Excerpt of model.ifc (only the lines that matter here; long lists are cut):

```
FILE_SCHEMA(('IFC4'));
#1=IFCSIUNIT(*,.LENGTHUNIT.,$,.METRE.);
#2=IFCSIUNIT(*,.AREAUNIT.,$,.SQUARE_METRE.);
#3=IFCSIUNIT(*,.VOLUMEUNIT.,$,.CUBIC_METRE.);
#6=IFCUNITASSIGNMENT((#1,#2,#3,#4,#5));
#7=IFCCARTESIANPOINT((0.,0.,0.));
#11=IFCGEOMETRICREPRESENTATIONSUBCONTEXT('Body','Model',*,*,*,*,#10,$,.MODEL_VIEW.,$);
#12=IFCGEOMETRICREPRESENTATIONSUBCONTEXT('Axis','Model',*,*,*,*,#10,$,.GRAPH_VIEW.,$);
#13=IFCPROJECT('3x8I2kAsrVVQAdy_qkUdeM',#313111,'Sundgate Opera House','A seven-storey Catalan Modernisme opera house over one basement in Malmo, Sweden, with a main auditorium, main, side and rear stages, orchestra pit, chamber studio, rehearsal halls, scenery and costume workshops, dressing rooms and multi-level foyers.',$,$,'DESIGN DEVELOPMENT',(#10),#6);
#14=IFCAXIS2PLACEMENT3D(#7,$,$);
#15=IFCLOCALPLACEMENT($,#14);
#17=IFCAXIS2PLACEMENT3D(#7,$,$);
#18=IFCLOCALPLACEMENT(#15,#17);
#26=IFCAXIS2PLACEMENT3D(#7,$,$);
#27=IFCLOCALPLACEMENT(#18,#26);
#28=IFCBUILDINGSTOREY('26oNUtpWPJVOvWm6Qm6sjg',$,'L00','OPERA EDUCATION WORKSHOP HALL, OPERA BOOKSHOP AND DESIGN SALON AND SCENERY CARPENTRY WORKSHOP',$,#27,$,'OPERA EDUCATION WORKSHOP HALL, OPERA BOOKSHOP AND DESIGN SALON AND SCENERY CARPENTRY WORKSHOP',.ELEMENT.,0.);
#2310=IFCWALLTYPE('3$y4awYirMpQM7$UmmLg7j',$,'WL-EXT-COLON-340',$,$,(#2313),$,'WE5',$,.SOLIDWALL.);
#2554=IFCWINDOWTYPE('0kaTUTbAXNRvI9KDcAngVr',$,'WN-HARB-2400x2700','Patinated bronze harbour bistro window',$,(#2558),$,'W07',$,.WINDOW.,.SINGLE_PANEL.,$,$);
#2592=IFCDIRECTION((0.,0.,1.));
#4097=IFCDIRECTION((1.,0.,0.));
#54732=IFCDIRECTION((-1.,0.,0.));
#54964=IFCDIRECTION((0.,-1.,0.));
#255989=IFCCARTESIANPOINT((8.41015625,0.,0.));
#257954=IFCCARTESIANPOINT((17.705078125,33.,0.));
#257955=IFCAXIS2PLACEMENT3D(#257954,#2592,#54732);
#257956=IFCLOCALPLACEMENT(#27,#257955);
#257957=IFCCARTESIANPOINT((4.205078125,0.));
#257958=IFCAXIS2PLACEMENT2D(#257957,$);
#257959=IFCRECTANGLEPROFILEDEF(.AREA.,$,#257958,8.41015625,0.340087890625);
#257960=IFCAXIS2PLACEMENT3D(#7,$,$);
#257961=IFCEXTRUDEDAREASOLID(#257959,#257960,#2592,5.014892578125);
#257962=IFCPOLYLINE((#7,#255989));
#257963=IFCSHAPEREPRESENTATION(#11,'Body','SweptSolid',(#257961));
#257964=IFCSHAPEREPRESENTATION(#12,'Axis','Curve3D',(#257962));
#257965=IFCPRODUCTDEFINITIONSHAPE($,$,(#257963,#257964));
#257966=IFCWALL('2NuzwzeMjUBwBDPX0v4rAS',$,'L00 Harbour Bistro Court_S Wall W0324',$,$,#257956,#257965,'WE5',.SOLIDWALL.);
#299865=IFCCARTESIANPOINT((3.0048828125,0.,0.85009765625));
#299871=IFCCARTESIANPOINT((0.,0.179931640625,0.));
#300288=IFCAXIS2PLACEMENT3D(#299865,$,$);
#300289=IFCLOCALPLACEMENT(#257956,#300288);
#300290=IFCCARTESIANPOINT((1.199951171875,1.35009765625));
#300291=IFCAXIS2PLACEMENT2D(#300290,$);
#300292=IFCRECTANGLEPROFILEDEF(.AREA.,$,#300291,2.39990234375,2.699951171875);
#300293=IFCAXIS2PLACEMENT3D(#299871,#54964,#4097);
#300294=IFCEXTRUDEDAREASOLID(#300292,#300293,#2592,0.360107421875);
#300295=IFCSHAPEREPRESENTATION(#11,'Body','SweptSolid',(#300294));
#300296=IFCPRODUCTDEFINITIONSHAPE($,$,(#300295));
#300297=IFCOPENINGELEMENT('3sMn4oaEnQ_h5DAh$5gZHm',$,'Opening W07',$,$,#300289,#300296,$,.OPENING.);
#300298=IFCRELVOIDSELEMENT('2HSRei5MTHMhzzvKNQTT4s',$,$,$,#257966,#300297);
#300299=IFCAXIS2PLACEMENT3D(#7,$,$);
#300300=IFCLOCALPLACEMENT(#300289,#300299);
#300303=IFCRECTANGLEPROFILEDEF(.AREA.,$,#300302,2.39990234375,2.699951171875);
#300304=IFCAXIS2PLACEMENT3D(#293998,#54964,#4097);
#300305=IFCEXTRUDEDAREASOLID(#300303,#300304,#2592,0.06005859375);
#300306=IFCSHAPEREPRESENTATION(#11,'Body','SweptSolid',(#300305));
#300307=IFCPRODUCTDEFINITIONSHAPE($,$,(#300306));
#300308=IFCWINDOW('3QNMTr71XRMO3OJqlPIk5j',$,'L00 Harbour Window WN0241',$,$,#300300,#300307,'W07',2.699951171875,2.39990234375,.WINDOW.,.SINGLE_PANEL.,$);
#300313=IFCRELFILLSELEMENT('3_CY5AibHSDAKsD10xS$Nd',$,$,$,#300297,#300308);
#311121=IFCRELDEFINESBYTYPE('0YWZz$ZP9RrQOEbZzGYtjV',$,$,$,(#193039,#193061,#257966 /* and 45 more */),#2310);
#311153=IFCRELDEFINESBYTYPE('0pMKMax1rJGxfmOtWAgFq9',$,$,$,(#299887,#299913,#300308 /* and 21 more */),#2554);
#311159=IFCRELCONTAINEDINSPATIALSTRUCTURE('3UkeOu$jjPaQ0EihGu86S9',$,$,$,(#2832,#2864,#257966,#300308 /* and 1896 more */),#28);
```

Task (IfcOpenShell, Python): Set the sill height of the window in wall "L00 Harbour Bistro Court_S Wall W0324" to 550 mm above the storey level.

```python
import numpy as np
import ifcopenshell
import ifcopenshell.api.geometry
import ifcopenshell.geom
import ifcopenshell.util.element
import ifcopenshell.util.placement
import ifcopenshell.util.shape
import ifcopenshell.util.unit

model = ifcopenshell.open("model.ifc")
unit_scale = ifcopenshell.util.unit.calculate_unit_scale(model)

window = model.by_guid("3QNMTr71XRMO3OJqlPIk5j")
opening = window.FillsVoids[0].RelatingOpeningElement
storey = ifcopenshell.util.element.get_container(window, ifc_class="IfcBuildingStorey")
level = ifcopenshell.util.placement.get_local_placement(storey.ObjectPlacement)[2, 3]

# The opening's origin need not be at the sill, so measure its lowest point.
shape = ifcopenshell.geom.create_shape(ifcopenshell.geom.settings(), opening)
bottom = ifcopenshell.util.shape.get_shape_bottom_elevation(shape, shape.geometry) / unit_scale
dz = level + 0.55 - bottom

shift = np.array([0.0, 0.0, dz])
# The window is placed relative to its opening, so it follows when the opening moves.
matrix = ifcopenshell.util.placement.get_local_placement(opening.ObjectPlacement)
matrix[:3, 3] += shift
ifcopenshell.api.geometry.edit_object_placement(
    model, product=opening, matrix=matrix, is_si=False, should_transform_children=True
)

print(f"moved by {dz * unit_scale:+.3f} m")

model.write("model_rev.ifc")
```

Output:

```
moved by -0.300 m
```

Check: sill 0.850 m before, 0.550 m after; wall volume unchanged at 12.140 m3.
